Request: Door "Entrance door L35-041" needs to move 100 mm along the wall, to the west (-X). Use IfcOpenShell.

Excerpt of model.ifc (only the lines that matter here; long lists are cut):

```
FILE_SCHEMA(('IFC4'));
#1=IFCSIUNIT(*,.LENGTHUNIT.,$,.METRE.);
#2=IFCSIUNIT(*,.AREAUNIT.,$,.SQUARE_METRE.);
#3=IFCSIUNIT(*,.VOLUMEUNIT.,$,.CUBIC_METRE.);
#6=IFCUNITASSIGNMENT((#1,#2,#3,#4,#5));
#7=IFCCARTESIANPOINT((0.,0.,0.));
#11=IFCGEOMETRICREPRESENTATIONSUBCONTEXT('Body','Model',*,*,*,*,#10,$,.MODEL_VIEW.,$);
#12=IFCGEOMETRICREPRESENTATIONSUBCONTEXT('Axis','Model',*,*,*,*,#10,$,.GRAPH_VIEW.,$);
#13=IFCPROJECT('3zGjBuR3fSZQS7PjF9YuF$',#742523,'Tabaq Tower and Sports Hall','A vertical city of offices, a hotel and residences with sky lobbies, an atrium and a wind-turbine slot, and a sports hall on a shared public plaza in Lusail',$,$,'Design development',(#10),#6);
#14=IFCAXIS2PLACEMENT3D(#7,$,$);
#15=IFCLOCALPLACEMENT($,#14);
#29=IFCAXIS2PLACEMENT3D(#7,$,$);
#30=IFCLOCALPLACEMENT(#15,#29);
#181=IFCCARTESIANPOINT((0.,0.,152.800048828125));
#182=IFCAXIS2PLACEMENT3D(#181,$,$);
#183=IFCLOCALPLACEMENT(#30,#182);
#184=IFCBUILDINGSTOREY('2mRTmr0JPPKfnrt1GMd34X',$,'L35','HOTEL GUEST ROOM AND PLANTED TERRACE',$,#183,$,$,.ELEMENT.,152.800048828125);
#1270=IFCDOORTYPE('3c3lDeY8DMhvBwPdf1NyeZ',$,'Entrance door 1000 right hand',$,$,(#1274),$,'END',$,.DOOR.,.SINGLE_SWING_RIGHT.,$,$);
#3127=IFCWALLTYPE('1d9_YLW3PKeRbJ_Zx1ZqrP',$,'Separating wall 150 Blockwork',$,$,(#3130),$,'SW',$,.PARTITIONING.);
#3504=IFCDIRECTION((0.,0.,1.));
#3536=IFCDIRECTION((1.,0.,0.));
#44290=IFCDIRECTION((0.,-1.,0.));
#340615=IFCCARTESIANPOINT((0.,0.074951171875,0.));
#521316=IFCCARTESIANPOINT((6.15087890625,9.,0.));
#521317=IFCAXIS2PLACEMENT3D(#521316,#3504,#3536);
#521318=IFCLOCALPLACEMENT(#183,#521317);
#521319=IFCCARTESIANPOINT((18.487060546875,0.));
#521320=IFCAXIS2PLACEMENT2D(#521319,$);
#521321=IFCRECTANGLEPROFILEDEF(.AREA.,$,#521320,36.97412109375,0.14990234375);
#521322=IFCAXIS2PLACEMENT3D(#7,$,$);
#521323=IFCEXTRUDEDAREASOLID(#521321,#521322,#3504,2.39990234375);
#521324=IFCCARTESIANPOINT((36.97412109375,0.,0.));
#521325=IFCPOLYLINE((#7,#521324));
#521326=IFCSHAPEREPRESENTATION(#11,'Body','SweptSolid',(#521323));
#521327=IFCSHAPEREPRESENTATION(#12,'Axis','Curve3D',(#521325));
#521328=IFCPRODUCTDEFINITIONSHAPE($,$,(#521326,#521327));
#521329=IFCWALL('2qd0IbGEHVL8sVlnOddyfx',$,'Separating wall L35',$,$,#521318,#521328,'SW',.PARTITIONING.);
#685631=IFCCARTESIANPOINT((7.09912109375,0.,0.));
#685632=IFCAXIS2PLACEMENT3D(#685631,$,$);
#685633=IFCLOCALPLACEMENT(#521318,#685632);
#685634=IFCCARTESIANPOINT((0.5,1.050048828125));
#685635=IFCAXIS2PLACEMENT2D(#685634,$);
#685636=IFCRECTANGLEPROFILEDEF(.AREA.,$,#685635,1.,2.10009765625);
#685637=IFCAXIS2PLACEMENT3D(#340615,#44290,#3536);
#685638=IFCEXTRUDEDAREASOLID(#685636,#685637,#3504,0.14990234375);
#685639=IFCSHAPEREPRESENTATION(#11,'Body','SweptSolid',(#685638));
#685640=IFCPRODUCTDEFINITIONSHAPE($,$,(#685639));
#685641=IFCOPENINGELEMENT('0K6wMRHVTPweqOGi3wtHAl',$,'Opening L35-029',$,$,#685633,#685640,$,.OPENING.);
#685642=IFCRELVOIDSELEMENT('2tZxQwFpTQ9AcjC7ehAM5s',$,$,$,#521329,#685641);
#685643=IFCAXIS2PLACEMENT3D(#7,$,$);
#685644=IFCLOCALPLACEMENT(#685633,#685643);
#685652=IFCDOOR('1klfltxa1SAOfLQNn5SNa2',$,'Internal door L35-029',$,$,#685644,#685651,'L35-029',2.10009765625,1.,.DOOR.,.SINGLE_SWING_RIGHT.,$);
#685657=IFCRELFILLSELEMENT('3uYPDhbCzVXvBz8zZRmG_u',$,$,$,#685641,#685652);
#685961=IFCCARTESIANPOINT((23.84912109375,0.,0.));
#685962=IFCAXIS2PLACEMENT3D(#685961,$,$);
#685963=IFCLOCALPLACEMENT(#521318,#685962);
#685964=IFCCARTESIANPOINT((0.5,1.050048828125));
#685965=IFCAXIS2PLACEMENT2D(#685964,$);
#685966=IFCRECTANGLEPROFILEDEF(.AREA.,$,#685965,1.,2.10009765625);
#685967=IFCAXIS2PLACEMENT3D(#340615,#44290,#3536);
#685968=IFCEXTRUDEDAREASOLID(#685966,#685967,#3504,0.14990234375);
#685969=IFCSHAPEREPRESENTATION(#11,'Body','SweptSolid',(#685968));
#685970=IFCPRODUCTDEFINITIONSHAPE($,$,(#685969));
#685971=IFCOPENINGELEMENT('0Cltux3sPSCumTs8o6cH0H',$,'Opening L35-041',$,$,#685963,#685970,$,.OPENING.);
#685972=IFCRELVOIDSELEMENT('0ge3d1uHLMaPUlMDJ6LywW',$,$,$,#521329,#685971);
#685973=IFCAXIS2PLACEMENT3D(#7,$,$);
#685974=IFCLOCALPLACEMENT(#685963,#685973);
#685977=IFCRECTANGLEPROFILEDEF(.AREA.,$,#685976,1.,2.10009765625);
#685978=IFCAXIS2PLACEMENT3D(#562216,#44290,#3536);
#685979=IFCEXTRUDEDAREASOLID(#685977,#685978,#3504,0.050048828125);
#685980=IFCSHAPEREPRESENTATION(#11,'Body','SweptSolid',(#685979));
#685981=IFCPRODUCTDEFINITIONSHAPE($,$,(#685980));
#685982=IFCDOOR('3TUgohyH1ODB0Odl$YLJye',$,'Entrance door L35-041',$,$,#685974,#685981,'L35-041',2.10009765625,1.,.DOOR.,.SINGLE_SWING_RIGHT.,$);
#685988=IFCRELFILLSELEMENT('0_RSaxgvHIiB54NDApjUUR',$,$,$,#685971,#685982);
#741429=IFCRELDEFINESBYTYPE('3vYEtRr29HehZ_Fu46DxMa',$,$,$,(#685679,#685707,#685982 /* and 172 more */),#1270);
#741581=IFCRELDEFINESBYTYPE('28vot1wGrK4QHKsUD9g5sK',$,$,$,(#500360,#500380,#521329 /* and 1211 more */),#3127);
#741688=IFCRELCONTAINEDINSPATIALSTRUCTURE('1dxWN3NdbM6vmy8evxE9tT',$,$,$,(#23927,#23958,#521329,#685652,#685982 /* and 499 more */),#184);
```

```python
import ifcopenshell
import ifcopenshell.api.geometry
import ifcopenshell.util.placement
import ifcopenshell.util.unit

model = ifcopenshell.open("model.ifc")
unit_scale = ifcopenshell.util.unit.calculate_unit_scale(model)

door = model.by_id(685982)
opening = door.FillsVoids[0].RelatingOpeningElement
wall = opening.VoidsElements[0].RelatingBuildingElement

wall_matrix = ifcopenshell.util.placement.get_local_placement(wall.ObjectPlacement)
shift = wall_matrix[:3, 0] * -0.1 / unit_scale
before = ifcopenshell.util.placement.get_local_placement(door.ObjectPlacement)[:3, 3].copy()

# The door is placed relative to its opening, so it follows when the opening moves.
matrix = ifcopenshell.util.placement.get_local_placement(opening.ObjectPlacement)
matrix[:3, 3] += shift
ifcopenshell.api.geometry.edit_object_placement(
    model, product=opening, matrix=matrix, is_si=False, should_transform_children=True
)

after = ifcopenshell.util.placement.get_local_placement(door.ObjectPlacement)[:3, 3]
print("door moved by", (after - before).round(3) + 0.0)

model.write("model_v2.ifc")
```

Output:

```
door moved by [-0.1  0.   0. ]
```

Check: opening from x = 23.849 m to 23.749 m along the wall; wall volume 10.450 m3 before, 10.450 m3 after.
